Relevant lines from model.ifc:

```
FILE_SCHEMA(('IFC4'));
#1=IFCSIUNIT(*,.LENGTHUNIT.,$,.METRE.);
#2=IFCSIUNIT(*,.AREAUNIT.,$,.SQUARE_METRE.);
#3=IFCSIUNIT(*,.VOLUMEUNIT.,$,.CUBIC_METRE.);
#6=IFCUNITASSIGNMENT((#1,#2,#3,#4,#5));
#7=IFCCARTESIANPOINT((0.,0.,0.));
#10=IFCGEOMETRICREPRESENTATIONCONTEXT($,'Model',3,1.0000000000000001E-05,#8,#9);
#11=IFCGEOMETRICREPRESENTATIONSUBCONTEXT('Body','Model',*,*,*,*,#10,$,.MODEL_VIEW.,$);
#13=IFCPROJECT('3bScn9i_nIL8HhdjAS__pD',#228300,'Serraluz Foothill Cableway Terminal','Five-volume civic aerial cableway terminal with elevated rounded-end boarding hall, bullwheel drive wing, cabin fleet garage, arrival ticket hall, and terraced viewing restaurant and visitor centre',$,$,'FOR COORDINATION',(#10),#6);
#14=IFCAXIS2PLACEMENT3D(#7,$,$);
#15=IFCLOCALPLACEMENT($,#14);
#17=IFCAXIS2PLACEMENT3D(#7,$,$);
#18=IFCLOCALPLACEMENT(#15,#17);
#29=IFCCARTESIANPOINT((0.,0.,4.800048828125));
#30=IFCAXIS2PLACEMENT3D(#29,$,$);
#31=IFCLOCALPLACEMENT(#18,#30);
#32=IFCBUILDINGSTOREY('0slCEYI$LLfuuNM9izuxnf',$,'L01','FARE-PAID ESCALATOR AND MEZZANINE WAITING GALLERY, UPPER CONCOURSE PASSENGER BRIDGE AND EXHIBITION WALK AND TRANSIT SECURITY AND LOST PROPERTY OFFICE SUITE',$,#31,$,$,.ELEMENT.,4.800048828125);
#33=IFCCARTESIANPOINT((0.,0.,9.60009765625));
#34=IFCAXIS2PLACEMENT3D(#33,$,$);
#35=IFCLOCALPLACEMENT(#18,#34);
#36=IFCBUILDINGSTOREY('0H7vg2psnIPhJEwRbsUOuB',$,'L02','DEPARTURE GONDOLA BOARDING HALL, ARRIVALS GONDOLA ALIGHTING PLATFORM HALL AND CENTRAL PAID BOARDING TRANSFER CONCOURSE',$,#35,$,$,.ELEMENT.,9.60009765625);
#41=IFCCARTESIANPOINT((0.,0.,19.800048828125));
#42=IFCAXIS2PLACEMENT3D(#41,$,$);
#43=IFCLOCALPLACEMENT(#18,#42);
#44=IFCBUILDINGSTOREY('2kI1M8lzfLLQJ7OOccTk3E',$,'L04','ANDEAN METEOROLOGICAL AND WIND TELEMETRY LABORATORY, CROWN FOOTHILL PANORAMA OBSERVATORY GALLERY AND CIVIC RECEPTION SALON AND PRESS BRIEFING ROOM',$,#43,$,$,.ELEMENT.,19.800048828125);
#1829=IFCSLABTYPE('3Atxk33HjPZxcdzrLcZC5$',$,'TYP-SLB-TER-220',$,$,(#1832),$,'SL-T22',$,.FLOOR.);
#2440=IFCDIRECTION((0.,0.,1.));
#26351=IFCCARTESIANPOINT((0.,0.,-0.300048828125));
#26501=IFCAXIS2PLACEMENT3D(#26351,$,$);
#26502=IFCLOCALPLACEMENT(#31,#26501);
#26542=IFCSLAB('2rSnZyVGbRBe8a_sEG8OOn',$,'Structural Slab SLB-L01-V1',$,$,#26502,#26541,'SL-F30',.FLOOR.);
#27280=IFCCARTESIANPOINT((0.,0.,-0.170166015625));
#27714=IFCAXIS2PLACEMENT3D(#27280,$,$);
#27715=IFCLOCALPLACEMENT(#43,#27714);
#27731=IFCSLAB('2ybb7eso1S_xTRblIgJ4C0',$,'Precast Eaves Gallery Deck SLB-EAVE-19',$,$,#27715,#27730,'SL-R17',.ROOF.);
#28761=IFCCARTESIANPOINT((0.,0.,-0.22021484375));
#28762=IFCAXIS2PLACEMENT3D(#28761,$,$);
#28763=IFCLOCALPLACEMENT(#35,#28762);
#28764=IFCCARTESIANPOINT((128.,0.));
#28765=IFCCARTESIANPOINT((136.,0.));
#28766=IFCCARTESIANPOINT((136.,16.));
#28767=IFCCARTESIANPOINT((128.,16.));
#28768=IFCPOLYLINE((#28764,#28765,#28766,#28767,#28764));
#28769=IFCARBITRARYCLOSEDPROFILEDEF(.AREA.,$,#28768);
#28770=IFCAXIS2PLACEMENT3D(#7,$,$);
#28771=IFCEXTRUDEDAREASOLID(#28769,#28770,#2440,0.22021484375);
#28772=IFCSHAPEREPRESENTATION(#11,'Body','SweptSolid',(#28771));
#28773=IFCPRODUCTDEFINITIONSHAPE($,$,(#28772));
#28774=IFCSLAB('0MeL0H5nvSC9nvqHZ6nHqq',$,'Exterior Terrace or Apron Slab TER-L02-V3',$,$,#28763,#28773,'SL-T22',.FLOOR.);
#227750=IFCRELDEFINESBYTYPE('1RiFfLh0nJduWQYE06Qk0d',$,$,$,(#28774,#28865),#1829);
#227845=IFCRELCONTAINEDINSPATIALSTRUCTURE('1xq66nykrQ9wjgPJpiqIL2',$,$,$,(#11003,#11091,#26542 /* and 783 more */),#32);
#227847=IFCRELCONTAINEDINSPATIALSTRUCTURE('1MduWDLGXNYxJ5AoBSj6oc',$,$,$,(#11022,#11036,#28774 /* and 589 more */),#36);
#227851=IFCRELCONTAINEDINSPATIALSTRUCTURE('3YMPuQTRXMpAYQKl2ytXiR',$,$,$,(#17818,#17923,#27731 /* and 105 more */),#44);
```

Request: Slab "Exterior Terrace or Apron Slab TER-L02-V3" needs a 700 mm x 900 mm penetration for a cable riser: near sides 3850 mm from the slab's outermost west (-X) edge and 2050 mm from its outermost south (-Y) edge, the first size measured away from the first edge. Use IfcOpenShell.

```python
import numpy as np
import ifcopenshell
import ifcopenshell.api.feature
import ifcopenshell.api.geometry
import ifcopenshell.api.root
import ifcopenshell.geom
import ifcopenshell.util.placement
import ifcopenshell.util.representation
import ifcopenshell.util.shape
import ifcopenshell.util.unit

model = ifcopenshell.open("model.ifc")
unit_scale = ifcopenshell.util.unit.calculate_unit_scale(model)
settings = ifcopenshell.geom.settings()


def volume(element):
    """Net volume in cubic metres, openings subtracted."""
    shape = ifcopenshell.geom.create_shape(settings, element)
    return ifcopenshell.util.shape.get_volume(shape.geometry)


slab = model.by_guid("0MeL0H5nvSC9nvqHZ6nHqq")
before = volume(slab)

# Extent in the slab's own axes, in metres. The edges named are its -X and -Y sides.
slab_shape = ifcopenshell.geom.create_shape(settings, slab)
vertices = ifcopenshell.util.shape.get_vertices(slab_shape.geometry)
x_min, y_min, bottom = vertices.min(axis=0)
top = vertices[:, 2].max()

opening = ifcopenshell.api.root.create_entity(model, ifc_class="IfcOpeningElement", name="Cable riser opening", predefined_type="OPENING")
context = ifcopenshell.util.representation.get_context(model, "Model", "Body", "MODEL_VIEW")
width, depth = 0.7, 0.9
outline = [(0.0, 0.0), (width, 0.0), (width, depth), (0.0, depth), (0.0, 0.0)]
# Overshoot both faces by 50 mm so the cut is clean.
shape = ifcopenshell.api.geometry.add_slab_representation(
    model, context=context, depth=top - bottom + 0.1, polyline=outline
)
ifcopenshell.api.geometry.assign_representation(model, product=opening, representation=shape)

matrix = ifcopenshell.util.placement.get_local_placement(slab.ObjectPlacement)
matrix[:, 3] = matrix @ np.append(np.array([x_min + 3.85, y_min + 2.05, bottom - 0.05]) / unit_scale, 1.0)
ifcopenshell.api.geometry.edit_object_placement(model, product=opening, matrix=matrix, is_si=False)
ifcopenshell.api.feature.add_feature(model, feature=opening, element=slab)

after = volume(slab)

print(f"slab volume {before:.3f} -> {after:.3f} m3")

model.write("model_updated.ifc")
```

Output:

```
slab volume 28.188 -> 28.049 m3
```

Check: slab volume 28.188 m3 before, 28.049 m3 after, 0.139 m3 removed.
